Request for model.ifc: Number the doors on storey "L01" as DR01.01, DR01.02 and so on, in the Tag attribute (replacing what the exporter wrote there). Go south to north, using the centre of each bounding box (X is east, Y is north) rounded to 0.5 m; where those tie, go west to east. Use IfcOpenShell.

First a look at what the model holds.

```python
import ifcopenshell
import ifcopenshell.util.element
import ifcopenshell.util.placement

model = ifcopenshell.open("model.ifc")
print(model.schema)
storey = next(s for s in model.by_type("IfcBuildingStorey") if s.Name == "L01")
doors = [e for e in ifcopenshell.util.element.get_decomposition(storey) if e.is_a("IfcDoor")]
for e in sorted(doors, key=lambda e: e.id()):
    origin = ifcopenshell.util.placement.get_local_placement(e.ObjectPlacement)[:3, 3]
    print(e.id(), e.Tag, e.Name, origin.round(2) + 0.0, sep=" | ")
```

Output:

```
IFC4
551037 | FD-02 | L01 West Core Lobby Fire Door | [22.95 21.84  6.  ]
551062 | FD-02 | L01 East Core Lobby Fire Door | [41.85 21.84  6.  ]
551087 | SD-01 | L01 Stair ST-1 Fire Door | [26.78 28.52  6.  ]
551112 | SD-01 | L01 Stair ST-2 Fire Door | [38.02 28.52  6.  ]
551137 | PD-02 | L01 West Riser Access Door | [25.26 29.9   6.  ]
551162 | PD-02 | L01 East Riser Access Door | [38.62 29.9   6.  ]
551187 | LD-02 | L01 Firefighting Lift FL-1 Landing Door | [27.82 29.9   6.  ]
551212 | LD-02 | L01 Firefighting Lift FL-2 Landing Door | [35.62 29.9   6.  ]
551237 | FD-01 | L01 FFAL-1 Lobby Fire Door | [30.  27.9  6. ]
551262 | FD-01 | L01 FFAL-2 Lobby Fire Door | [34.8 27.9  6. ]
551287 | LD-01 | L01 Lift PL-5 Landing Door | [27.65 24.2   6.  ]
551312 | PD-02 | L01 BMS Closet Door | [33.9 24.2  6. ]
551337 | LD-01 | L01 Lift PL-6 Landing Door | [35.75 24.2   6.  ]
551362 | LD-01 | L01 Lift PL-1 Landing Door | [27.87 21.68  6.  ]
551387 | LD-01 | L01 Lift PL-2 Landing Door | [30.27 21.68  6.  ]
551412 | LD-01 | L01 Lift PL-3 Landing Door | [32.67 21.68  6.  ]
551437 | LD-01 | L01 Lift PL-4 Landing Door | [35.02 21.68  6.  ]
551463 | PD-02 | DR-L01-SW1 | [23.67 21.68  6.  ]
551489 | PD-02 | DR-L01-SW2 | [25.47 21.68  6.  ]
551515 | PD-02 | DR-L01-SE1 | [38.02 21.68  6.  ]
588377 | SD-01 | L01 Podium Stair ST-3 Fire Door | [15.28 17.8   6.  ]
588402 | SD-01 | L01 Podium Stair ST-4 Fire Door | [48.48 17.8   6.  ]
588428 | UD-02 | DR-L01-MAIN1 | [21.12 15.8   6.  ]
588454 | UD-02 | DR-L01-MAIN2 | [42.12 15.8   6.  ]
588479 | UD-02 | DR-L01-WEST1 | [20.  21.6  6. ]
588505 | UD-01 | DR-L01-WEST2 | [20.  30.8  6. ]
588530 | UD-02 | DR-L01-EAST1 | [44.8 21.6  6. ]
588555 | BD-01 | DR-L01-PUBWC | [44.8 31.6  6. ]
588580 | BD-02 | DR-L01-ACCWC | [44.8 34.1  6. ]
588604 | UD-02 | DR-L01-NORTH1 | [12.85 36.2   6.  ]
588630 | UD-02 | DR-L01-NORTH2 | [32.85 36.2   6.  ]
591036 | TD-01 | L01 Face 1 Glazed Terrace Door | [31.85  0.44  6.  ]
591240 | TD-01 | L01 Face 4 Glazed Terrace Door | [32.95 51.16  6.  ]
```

```python
import ifcopenshell
import ifcopenshell.geom
import ifcopenshell.util.element
import ifcopenshell.util.shape

model = ifcopenshell.open("model.ifc")
settings = ifcopenshell.geom.settings()
settings.set("use-world-coords", True)


def centre(element):
    shape = ifcopenshell.geom.create_shape(settings, element)
    return ifcopenshell.util.shape.get_bbox_centroid(shape.geometry)


storey = next(s for s in model.by_type("IfcBuildingStorey") if s.Name == "L01")
doors = [e for e in ifcopenshell.util.element.get_decomposition(storey) if e.is_a("IfcDoor")]

# Insertion points can sit at a corner or the storey origin, so sort by the geometry (in metres).
centres = {e: centre(e) for e in doors}
doors.sort(key=lambda e: (round(centres[e][1] / 0.5), centres[e][0]))

for i, e in enumerate(doors, start=1):
    number = f"DR01.{i:02d}"
    e.Tag = number
    print(e.id(), number)

model.write("model-out.ifc")
```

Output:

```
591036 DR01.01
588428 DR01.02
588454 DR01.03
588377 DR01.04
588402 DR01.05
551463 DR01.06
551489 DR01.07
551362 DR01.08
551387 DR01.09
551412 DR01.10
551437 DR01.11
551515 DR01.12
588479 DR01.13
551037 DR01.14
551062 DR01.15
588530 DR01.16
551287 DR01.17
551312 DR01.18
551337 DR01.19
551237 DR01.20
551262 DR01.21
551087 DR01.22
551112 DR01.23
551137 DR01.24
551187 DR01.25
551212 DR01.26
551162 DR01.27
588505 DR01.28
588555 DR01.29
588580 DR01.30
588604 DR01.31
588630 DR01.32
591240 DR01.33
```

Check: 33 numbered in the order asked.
